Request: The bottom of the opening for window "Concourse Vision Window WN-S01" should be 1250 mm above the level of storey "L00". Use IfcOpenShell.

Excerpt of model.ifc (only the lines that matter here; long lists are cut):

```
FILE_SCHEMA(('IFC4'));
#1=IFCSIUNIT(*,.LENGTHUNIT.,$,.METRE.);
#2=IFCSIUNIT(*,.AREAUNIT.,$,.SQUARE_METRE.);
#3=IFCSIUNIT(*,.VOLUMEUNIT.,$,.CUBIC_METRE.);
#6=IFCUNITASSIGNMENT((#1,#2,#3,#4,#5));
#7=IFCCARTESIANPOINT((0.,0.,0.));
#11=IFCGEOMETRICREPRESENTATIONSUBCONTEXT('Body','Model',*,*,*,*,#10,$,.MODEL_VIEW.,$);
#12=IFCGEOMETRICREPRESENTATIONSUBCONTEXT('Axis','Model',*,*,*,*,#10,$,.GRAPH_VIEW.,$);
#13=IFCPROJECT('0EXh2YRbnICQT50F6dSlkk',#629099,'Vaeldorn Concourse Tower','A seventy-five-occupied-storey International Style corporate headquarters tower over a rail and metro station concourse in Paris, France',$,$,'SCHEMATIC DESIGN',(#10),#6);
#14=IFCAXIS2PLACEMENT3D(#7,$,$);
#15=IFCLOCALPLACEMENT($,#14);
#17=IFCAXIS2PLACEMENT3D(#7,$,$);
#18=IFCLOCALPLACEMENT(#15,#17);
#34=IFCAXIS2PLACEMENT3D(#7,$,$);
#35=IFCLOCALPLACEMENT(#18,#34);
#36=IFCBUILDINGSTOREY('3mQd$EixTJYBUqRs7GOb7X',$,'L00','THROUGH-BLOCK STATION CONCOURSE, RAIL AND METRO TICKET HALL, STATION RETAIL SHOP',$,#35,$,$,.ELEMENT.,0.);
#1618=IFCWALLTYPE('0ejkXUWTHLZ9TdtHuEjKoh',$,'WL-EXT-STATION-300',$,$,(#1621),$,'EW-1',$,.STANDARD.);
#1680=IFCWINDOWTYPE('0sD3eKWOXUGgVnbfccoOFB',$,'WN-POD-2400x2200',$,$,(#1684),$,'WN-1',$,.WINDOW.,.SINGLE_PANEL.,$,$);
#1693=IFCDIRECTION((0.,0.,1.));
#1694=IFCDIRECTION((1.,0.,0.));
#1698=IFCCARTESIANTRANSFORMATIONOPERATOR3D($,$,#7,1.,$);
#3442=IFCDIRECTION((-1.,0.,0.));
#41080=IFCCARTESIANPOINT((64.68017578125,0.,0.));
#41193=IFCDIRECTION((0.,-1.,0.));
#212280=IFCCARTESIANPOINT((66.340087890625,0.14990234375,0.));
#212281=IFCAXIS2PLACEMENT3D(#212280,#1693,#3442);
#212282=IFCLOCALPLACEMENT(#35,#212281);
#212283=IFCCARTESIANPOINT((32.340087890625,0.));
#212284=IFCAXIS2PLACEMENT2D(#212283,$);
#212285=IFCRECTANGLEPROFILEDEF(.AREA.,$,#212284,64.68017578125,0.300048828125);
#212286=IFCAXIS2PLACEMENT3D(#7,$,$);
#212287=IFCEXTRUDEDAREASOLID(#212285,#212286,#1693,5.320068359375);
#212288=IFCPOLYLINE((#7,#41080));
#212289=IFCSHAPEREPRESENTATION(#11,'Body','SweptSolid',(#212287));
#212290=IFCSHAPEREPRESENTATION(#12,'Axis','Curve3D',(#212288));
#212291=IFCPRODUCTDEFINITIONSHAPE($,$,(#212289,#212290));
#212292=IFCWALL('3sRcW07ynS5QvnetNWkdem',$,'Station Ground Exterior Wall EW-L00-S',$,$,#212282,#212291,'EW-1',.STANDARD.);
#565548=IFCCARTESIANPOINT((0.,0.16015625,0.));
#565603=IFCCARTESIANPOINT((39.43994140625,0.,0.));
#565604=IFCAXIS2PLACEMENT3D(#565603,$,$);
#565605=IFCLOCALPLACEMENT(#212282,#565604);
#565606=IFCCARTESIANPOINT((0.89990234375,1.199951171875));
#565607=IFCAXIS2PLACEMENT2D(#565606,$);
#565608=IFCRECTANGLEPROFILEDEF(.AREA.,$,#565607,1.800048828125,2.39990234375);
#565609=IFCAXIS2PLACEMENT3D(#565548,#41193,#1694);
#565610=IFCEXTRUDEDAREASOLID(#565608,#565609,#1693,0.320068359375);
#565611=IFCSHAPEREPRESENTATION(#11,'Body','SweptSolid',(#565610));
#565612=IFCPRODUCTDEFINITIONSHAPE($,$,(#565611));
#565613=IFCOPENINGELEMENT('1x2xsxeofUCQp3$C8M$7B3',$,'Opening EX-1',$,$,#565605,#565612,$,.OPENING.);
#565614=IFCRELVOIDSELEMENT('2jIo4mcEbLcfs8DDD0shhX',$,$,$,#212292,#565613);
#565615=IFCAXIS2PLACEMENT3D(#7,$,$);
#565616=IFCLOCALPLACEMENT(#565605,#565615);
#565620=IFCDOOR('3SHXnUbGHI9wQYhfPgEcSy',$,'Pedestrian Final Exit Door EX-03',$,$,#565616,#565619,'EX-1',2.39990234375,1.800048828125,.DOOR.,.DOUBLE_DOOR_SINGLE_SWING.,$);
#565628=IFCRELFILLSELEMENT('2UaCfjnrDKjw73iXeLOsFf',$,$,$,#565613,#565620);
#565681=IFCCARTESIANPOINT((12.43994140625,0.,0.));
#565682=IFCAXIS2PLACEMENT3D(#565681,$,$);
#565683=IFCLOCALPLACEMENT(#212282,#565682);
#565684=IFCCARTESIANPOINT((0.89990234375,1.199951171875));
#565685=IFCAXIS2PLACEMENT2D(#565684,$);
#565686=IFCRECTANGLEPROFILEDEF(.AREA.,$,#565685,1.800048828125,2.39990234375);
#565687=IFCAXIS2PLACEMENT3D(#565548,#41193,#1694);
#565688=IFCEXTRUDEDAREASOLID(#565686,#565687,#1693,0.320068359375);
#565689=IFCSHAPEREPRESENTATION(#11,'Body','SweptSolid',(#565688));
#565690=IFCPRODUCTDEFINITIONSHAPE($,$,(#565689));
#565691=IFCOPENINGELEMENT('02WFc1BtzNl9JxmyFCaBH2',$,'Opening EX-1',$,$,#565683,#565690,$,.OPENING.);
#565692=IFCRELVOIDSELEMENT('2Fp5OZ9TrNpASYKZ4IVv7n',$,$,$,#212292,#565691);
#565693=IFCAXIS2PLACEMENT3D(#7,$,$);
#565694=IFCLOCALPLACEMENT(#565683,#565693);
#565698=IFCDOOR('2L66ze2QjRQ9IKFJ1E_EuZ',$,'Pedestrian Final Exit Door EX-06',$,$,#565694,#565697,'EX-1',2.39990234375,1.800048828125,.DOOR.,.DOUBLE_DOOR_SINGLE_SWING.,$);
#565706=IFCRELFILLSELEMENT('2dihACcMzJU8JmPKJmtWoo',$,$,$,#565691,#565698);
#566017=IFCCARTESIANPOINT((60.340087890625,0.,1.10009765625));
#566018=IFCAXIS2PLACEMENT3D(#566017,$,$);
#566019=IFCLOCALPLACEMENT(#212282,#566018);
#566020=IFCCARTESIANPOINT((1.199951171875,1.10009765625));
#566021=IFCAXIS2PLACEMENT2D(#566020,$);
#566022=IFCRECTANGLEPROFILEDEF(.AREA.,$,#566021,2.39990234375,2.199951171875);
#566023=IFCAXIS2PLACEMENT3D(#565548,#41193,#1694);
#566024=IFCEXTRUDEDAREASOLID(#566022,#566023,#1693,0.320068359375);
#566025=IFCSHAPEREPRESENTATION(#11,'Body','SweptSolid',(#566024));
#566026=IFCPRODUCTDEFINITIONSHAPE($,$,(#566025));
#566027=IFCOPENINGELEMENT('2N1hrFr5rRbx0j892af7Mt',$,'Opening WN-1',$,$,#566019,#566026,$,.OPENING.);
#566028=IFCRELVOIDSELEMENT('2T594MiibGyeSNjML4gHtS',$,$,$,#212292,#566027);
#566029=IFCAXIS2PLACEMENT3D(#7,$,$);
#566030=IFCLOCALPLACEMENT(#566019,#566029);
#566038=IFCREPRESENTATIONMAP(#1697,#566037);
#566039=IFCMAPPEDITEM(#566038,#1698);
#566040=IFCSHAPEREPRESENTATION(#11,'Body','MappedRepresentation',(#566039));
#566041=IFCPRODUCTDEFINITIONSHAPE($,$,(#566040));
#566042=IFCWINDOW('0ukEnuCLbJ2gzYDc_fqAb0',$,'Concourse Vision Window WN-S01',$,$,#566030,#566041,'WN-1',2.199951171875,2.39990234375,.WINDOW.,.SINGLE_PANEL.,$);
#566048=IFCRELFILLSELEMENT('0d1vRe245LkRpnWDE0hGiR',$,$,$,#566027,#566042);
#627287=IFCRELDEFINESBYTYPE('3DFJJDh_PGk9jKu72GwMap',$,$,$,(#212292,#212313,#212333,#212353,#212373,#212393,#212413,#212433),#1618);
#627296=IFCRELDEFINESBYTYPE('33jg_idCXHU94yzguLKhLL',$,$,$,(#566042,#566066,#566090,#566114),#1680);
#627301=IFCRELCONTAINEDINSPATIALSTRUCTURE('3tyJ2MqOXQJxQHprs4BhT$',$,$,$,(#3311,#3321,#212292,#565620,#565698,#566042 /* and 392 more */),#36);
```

```python
import numpy as np
import ifcopenshell
import ifcopenshell.api.geometry
import ifcopenshell.geom
import ifcopenshell.util.element
import ifcopenshell.util.placement
import ifcopenshell.util.shape
import ifcopenshell.util.unit

model = ifcopenshell.open("model.ifc")
unit_scale = ifcopenshell.util.unit.calculate_unit_scale(model)

window = model.by_id(566042)
opening = window.FillsVoids[0].RelatingOpeningElement
storey = ifcopenshell.util.element.get_container(window, ifc_class="IfcBuildingStorey")
level = ifcopenshell.util.placement.get_local_placement(storey.ObjectPlacement)[2, 3]

# The opening's origin need not be at the sill, so measure its lowest point.
shape = ifcopenshell.geom.create_shape(ifcopenshell.geom.settings(), opening)
bottom = ifcopenshell.util.shape.get_shape_bottom_elevation(shape, shape.geometry) / unit_scale
dz = level + 1.25 / unit_scale - bottom

shift = np.array([0.0, 0.0, dz])
# The window is placed relative to its opening, so it follows when the opening moves.
matrix = ifcopenshell.util.placement.get_local_placement(opening.ObjectPlacement)
matrix[:3, 3] += shift
ifcopenshell.api.geometry.edit_object_placement(
    model, product=opening, matrix=matrix, is_si=False, should_transform_children=True
)

print(f"moved by {dz * unit_scale:+.3f} m")

model.write("model_edited.ifc")
```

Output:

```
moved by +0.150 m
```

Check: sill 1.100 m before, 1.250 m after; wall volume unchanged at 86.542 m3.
